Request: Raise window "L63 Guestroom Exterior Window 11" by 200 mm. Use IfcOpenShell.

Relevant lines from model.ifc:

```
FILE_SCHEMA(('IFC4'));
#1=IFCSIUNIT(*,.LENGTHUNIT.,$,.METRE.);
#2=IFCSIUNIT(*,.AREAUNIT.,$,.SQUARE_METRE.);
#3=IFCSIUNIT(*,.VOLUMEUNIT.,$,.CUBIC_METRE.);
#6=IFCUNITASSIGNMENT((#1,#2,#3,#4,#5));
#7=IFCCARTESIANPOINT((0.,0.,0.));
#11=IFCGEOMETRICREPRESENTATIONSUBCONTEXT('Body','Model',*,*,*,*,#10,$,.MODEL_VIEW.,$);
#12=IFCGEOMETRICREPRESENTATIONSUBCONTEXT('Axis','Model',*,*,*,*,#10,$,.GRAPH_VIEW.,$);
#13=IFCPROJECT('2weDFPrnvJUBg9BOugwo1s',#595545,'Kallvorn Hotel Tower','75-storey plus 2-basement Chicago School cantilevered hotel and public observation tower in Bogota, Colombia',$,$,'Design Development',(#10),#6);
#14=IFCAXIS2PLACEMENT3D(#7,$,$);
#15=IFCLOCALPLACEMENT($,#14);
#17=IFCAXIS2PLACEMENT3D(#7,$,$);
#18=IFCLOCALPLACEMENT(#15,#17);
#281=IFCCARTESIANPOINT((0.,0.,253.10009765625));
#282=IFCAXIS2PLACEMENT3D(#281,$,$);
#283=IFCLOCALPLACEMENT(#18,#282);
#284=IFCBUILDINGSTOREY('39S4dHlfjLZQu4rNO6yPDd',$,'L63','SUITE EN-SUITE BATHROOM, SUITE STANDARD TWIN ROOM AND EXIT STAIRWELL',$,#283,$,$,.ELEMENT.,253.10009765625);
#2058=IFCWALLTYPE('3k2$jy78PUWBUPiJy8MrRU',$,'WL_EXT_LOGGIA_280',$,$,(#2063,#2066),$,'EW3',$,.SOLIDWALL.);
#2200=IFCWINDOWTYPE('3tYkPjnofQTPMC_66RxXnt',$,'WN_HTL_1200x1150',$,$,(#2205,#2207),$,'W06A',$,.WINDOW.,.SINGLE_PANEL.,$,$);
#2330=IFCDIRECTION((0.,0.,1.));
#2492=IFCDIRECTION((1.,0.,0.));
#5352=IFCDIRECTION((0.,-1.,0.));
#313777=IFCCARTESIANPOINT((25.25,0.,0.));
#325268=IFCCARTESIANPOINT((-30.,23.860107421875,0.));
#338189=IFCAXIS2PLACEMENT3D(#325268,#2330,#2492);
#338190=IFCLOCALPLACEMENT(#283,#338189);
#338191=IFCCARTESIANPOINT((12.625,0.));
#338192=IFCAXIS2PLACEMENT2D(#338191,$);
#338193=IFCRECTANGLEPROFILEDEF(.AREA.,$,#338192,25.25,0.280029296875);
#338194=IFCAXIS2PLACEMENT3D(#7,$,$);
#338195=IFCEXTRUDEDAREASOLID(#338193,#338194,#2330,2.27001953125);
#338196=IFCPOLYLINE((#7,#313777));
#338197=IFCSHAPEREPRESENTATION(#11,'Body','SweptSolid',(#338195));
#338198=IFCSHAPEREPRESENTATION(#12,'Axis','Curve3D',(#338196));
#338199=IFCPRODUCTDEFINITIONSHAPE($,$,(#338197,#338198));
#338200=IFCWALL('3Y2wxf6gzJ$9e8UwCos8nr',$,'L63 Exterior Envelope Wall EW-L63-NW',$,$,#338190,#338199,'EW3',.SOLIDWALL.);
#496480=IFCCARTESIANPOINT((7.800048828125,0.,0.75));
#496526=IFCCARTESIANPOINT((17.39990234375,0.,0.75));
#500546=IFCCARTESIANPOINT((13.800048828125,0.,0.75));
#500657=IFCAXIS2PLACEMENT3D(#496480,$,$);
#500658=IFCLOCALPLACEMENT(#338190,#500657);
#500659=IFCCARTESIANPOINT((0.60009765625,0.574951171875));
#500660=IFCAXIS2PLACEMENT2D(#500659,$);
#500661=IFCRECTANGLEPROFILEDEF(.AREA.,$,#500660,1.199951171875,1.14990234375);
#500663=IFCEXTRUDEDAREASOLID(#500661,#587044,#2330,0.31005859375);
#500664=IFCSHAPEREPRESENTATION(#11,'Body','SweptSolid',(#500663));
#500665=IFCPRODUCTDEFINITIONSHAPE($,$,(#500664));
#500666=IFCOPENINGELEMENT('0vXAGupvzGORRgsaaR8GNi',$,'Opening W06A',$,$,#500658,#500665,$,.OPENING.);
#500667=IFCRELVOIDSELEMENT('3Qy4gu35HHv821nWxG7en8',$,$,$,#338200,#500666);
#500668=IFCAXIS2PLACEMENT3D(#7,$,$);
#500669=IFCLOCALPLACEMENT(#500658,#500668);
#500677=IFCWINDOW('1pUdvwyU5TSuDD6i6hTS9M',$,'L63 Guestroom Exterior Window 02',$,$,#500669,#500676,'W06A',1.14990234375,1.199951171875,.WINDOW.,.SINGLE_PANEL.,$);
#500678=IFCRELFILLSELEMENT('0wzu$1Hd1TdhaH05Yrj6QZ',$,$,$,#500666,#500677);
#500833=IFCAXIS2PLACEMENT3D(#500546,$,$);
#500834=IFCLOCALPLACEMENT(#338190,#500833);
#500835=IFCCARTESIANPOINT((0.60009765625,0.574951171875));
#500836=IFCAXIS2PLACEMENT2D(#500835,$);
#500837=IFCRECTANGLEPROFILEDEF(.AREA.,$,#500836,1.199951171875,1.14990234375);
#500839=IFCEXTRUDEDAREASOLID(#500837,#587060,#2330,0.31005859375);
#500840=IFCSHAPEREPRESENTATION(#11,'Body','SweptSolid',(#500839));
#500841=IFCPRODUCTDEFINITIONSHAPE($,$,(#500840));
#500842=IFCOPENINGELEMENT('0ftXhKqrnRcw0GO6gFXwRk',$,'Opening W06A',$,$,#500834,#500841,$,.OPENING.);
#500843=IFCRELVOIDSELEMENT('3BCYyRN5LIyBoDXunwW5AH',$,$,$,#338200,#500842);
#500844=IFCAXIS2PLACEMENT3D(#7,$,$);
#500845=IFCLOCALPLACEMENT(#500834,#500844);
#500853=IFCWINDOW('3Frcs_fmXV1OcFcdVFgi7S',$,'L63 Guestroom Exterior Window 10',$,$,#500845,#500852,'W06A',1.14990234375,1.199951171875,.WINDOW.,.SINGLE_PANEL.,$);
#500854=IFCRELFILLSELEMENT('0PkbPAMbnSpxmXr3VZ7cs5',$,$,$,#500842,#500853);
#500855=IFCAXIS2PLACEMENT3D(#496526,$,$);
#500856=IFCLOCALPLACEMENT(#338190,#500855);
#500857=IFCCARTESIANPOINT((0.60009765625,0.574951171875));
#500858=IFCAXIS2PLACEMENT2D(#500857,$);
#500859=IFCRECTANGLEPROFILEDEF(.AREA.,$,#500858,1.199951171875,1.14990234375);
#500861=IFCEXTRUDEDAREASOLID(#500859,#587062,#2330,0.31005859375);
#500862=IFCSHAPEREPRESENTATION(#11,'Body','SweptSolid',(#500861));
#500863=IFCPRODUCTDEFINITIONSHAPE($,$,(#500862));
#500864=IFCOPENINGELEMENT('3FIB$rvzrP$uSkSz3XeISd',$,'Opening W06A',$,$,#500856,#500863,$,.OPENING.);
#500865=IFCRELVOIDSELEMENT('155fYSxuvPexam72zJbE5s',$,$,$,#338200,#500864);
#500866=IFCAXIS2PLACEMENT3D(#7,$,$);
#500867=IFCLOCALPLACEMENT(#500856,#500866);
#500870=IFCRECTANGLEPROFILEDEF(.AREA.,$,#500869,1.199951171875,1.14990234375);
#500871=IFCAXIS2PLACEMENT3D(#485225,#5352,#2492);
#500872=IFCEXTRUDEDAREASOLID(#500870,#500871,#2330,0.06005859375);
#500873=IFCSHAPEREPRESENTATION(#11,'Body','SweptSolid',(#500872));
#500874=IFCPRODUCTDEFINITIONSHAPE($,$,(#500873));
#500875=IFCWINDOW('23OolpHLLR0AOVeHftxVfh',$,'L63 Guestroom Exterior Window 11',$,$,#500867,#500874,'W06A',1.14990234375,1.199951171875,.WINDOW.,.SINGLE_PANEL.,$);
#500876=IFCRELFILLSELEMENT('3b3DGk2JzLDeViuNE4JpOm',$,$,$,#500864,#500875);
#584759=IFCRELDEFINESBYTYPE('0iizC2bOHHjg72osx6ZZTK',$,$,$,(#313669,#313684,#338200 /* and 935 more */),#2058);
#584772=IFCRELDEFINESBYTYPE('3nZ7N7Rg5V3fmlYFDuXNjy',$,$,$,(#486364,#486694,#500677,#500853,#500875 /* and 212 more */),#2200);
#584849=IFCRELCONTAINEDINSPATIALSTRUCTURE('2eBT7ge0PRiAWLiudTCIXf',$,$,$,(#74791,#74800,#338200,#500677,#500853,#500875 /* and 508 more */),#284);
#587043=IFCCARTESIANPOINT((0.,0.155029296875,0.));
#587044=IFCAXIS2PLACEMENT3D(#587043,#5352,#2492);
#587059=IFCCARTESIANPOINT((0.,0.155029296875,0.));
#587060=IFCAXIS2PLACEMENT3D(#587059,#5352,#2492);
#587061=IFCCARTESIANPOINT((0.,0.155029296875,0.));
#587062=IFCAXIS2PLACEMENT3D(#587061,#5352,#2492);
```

```python
import numpy as np
import ifcopenshell
import ifcopenshell.api.geometry
import ifcopenshell.util.placement
import ifcopenshell.util.unit

model = ifcopenshell.open("model.ifc")
unit_scale = ifcopenshell.util.unit.calculate_unit_scale(model)

window = model.by_guid("23OolpHLLR0AOVeHftxVfh")
opening = window.FillsVoids[0].RelatingOpeningElement
dz = 0.2

shift = np.array([0.0, 0.0, dz])
# The window is placed relative to its opening, so it follows when the opening moves.
matrix = ifcopenshell.util.placement.get_local_placement(opening.ObjectPlacement)
matrix[:3, 3] += shift
ifcopenshell.api.geometry.edit_object_placement(
    model, product=opening, matrix=matrix, is_si=False, should_transform_children=True
)

print(f"moved by {dz * unit_scale:+.3f} m")

model.write("model_v2.ifc")
```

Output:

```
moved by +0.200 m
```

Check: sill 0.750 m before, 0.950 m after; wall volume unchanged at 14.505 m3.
